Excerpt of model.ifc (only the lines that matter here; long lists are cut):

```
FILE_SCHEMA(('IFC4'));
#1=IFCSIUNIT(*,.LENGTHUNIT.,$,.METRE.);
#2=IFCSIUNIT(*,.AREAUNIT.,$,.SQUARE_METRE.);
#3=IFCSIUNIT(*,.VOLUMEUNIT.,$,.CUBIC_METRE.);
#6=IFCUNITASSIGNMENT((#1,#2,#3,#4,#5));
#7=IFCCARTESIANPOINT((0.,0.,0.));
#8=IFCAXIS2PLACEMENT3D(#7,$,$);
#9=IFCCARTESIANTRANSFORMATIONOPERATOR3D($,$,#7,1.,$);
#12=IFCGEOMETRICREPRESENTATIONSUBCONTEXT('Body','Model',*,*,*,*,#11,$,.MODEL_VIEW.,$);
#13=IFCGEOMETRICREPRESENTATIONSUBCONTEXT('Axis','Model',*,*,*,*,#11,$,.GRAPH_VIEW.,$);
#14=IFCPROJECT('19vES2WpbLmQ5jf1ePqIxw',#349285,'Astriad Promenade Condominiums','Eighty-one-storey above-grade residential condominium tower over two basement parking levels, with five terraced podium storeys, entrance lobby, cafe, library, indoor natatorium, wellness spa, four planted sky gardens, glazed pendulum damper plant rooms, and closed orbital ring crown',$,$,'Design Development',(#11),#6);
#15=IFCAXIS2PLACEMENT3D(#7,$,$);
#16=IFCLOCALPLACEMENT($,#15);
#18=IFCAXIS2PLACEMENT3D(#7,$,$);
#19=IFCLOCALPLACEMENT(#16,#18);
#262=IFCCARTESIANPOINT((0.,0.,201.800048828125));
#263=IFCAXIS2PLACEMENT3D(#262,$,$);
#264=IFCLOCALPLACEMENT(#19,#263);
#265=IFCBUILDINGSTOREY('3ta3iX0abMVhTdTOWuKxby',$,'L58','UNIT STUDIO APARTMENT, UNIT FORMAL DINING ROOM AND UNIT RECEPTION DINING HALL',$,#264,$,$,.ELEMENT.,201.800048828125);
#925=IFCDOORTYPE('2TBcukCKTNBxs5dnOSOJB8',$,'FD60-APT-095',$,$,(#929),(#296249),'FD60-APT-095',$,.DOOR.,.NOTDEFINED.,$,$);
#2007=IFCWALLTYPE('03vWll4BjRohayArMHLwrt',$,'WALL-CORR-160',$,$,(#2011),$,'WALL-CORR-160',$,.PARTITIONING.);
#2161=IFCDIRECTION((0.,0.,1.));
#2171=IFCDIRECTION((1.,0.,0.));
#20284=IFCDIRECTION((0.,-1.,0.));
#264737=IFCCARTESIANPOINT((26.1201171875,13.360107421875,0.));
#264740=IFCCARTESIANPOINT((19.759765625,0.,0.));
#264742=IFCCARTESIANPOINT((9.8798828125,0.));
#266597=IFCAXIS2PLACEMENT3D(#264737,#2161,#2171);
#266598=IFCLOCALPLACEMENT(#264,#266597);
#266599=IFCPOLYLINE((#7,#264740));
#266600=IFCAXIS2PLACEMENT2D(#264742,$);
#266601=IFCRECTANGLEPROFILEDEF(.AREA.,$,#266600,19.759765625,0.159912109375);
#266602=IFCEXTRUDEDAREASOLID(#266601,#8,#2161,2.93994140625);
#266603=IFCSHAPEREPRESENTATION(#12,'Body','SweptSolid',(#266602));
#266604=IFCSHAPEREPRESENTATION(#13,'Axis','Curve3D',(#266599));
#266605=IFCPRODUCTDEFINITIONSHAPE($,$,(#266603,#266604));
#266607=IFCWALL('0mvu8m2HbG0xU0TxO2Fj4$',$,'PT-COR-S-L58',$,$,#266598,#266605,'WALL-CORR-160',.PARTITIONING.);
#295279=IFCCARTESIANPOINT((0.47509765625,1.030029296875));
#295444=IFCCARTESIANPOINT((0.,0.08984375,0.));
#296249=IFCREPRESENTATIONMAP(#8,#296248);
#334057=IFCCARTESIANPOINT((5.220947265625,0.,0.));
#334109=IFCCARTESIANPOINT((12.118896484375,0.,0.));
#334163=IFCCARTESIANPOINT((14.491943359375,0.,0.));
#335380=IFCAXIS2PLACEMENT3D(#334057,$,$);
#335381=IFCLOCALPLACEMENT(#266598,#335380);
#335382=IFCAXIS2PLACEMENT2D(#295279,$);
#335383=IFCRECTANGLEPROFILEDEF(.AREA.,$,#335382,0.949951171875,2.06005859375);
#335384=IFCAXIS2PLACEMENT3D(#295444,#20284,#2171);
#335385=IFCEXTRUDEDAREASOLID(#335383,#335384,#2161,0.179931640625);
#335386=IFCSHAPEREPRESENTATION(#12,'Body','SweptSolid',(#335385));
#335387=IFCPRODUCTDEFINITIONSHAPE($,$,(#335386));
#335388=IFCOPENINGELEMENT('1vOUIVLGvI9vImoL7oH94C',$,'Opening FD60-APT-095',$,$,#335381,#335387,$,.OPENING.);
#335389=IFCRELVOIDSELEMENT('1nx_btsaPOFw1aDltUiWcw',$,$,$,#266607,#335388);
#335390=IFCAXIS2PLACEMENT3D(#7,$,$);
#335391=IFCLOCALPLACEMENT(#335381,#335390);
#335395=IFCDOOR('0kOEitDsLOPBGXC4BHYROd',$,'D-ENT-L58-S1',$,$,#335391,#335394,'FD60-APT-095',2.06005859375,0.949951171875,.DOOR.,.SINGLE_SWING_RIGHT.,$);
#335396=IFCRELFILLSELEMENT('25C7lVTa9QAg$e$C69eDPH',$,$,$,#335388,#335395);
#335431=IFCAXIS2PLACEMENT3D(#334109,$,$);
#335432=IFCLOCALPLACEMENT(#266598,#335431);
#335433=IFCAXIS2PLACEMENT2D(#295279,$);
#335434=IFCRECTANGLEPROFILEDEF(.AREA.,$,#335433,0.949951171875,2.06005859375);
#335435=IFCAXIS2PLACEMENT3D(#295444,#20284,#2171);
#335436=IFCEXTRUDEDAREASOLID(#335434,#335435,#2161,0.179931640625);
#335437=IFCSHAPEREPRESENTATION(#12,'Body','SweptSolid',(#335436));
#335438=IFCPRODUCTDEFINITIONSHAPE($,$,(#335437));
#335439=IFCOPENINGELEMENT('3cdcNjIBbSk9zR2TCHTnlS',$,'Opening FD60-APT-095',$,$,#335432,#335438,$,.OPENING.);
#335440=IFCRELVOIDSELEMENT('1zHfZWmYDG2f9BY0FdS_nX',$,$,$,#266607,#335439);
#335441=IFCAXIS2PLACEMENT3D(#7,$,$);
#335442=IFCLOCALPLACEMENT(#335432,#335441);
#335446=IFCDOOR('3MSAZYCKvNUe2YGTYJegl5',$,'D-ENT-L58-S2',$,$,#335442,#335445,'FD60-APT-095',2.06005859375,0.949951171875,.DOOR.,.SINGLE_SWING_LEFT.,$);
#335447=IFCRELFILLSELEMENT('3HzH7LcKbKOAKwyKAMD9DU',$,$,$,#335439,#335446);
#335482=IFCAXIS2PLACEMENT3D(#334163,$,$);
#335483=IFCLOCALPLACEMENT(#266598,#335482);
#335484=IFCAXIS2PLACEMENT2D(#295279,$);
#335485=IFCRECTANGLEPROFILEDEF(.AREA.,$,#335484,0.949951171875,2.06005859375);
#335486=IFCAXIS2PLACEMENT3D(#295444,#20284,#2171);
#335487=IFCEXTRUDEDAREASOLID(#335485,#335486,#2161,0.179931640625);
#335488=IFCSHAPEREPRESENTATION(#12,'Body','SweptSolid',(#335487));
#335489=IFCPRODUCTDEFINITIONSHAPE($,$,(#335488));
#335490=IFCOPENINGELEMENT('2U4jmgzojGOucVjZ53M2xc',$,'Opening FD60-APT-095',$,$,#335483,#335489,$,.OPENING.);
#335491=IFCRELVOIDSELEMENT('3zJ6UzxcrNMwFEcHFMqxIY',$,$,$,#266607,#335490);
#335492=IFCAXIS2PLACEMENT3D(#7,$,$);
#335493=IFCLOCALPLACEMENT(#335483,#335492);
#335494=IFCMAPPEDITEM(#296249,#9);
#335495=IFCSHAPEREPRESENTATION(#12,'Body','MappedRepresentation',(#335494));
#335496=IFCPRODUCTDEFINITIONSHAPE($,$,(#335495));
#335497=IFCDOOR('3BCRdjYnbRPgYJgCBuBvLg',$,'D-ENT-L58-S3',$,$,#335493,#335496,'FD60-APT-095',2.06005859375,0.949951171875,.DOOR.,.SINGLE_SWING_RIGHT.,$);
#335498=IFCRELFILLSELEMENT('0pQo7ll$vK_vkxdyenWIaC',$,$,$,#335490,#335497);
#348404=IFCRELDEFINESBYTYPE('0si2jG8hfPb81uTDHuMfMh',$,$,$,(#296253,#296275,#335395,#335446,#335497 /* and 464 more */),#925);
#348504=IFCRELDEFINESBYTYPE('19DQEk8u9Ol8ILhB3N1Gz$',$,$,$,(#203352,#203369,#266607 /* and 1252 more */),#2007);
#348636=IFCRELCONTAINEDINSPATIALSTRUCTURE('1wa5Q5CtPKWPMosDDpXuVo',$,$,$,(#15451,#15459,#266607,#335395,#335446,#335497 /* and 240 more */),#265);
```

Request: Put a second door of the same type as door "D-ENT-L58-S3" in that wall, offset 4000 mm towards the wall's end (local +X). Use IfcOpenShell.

```python
import ifcopenshell
import ifcopenshell.api.feature
import ifcopenshell.api.geometry
import ifcopenshell.api.root
import ifcopenshell.geom
import ifcopenshell.util.element
import ifcopenshell.util.placement
import ifcopenshell.util.shape

model = ifcopenshell.open("model.ifc")
settings = ifcopenshell.geom.settings()


def volume(element):
    """Net volume in cubic metres, openings subtracted."""
    shape = ifcopenshell.geom.create_shape(settings, element)
    return ifcopenshell.util.shape.get_volume(shape.geometry)


door = model.by_guid("3BCRdjYnbRPgYJgCBuBvLg")
opening = door.FillsVoids[0].RelatingOpeningElement
wall = opening.VoidsElements[0].RelatingBuildingElement
before = volume(wall)
shift = ifcopenshell.util.placement.get_local_placement(wall.ObjectPlacement)[:3, 0] * 4.0

# copy_class copies the void relationship, type, container and properties, but no geometry.
new_opening = ifcopenshell.api.root.copy_class(model, product=opening)
new_opening.Representation = ifcopenshell.util.element.copy_deep(
    model, opening.Representation, exclude=["IfcGeometricRepresentationContext", "IfcRepresentationMap"]
)
new_door = ifcopenshell.api.root.copy_class(model, product=door)
new_door.Representation = ifcopenshell.util.element.copy_deep(
    model, door.Representation, exclude=["IfcGeometricRepresentationContext", "IfcRepresentationMap"]
)
new_door.Tag = None
ifcopenshell.api.feature.add_filling(model, opening=new_opening, element=new_door)

for old, new in ((opening, new_opening), (door, new_door)):
    matrix = ifcopenshell.util.placement.get_local_placement(old.ObjectPlacement)
    matrix[:3, 3] += shift
    ifcopenshell.api.geometry.edit_object_placement(model, product=new, matrix=matrix, is_si=False)

after = volume(wall)

print(f"wall volume {before:.3f} -> {after:.3f} m3")

model.write("model_rev.ifc")
```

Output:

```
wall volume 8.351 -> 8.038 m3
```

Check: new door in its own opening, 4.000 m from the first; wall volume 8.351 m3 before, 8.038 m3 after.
